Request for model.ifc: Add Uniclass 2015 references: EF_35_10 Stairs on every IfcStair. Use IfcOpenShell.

First a look at what the model holds.

```python
import ifcopenshell

model = ifcopenshell.open("model.ifc")
print(model.schema)
print("classifications:", [c.Name for c in model.by_type("IfcClassification")])
for ifc_class in ("IfcDoor", "IfcRoof", "IfcStair", "IfcWall", "IfcWindow"):
    print(ifc_class, len(model.by_type(ifc_class)))
```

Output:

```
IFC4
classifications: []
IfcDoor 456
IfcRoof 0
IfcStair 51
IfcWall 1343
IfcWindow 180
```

```python
import ifcopenshell
import ifcopenshell.api.classification

model = ifcopenshell.open("model.ifc")

system = ifcopenshell.api.classification.add_classification(model, classification="Uniclass 2015")

codes = {
    "IfcStair": ("EF_35_10", "Stairs"),
}
for ifc_class, (code, name) in codes.items():
    products = model.by_type(ifc_class)
    ifcopenshell.api.classification.add_reference(
        model, products=products, classification=system, identification=code, name=name
    )
    print(code, len(products))

model.write("model_v2.ifc")
```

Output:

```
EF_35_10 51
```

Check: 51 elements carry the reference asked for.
